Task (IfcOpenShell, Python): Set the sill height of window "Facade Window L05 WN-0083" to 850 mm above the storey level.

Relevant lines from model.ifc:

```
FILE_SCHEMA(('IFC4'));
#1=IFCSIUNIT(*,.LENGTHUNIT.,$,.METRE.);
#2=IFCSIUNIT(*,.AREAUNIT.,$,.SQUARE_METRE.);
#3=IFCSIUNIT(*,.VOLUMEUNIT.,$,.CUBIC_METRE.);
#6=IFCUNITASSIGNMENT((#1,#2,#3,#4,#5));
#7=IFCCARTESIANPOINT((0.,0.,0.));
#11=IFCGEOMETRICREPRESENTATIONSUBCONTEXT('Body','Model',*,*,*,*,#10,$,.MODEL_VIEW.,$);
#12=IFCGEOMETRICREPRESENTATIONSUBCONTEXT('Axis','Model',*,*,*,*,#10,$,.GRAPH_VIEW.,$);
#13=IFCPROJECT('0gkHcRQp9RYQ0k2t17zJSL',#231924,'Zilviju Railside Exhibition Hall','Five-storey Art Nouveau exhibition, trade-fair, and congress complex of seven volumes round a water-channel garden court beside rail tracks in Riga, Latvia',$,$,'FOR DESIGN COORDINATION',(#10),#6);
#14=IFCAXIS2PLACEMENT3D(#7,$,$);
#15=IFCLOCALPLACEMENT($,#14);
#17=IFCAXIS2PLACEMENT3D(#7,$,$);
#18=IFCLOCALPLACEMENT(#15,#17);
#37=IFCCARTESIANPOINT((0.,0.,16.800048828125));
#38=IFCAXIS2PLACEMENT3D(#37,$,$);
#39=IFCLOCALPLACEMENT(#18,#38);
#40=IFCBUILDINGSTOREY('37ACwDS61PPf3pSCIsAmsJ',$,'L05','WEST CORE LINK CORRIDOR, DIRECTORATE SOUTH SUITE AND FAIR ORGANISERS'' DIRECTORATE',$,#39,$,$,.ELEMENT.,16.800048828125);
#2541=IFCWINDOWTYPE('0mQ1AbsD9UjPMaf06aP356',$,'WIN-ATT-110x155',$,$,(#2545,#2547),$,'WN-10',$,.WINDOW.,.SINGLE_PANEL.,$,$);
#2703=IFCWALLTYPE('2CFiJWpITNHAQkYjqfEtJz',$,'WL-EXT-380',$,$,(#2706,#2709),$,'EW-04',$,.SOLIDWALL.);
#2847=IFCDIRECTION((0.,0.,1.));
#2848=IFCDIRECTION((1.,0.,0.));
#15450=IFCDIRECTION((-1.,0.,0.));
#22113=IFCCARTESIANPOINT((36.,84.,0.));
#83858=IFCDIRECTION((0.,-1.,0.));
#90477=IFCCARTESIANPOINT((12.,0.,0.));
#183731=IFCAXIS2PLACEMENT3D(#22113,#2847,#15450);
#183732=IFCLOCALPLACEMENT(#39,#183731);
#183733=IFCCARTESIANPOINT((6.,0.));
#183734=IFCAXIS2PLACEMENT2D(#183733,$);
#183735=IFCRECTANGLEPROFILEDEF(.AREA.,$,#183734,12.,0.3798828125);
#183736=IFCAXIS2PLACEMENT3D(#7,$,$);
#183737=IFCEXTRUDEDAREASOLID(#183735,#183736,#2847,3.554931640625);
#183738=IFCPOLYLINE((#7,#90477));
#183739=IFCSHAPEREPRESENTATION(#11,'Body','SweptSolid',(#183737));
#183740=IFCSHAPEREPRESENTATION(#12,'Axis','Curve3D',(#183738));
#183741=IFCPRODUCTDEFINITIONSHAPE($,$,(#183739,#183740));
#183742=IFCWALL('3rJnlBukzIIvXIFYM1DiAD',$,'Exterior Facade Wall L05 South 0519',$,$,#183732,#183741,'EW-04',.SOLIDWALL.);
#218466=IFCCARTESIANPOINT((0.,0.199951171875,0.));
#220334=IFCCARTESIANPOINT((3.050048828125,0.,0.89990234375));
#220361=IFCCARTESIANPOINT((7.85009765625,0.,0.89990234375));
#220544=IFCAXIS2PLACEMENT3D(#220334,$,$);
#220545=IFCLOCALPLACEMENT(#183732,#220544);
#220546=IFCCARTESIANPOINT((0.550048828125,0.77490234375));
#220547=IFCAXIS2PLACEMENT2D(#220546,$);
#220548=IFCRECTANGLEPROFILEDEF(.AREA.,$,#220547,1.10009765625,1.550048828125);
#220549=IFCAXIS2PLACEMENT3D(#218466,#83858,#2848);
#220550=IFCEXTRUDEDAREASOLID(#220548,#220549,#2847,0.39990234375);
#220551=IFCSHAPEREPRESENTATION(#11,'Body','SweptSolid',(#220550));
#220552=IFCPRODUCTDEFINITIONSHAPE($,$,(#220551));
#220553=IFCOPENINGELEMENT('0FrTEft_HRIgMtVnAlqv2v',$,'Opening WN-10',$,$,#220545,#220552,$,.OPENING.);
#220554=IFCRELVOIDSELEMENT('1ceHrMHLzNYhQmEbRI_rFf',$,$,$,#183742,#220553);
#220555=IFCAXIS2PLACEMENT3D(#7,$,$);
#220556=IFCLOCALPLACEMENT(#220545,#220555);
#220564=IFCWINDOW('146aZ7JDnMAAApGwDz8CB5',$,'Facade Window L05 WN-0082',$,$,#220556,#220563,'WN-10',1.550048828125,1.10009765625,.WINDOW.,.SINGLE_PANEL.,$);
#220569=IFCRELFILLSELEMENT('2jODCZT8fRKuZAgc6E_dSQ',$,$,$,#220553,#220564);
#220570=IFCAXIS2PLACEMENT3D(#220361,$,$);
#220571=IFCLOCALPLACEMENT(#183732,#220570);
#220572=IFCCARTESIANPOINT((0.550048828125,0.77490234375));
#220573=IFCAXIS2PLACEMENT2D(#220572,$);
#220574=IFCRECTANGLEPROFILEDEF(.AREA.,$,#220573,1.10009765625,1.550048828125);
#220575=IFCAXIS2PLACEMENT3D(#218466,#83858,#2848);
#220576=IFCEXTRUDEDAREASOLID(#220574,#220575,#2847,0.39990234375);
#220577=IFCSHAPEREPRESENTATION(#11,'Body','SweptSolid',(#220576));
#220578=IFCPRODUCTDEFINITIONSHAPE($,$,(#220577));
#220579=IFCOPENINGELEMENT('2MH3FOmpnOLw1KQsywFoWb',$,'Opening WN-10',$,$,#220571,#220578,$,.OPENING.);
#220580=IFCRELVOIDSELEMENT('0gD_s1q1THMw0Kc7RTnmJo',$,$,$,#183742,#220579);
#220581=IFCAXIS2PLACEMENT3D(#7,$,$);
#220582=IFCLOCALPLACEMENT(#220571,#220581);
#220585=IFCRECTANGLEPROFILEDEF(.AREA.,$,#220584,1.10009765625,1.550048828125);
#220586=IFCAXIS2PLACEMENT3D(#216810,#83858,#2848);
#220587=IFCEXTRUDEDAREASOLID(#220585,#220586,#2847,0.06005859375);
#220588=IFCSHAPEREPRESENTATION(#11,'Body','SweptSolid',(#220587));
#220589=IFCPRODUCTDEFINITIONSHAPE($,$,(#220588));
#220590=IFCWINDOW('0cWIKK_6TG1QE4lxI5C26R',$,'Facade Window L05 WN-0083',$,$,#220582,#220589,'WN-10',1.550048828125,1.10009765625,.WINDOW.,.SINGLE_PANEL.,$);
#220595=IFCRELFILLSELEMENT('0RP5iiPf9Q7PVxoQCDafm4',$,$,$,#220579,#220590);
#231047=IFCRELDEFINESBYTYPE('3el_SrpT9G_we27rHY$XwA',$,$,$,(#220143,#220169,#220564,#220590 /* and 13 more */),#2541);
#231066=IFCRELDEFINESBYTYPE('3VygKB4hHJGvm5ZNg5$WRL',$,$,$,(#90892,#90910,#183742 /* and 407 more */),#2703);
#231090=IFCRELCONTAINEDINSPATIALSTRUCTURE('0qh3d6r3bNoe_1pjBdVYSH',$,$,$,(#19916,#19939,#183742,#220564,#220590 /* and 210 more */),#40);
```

```python
import numpy as np
import ifcopenshell
import ifcopenshell.api.geometry
import ifcopenshell.geom
import ifcopenshell.util.element
import ifcopenshell.util.placement
import ifcopenshell.util.shape
import ifcopenshell.util.unit

model = ifcopenshell.open("model.ifc")
unit_scale = ifcopenshell.util.unit.calculate_unit_scale(model)

window = model.by_guid("0cWIKK_6TG1QE4lxI5C26R")
opening = window.FillsVoids[0].RelatingOpeningElement
storey = ifcopenshell.util.element.get_container(window, ifc_class="IfcBuildingStorey")
level = ifcopenshell.util.placement.get_local_placement(storey.ObjectPlacement)[2, 3]

# The opening's origin need not be at the sill, so measure its lowest point.
shape = ifcopenshell.geom.create_shape(ifcopenshell.geom.settings(), opening)
bottom = ifcopenshell.util.shape.get_shape_bottom_elevation(shape, shape.geometry) / unit_scale
dz = level + 0.85 / unit_scale - bottom

shift = np.array([0.0, 0.0, dz])
# The window is placed relative to its opening, so it follows when the opening moves.
matrix = ifcopenshell.util.placement.get_local_placement(opening.ObjectPlacement)
matrix[:3, 3] += shift
ifcopenshell.api.geometry.edit_object_placement(
    model, product=opening, matrix=matrix, is_si=False, should_transform_children=True
)

print(f"moved by {dz * unit_scale:+.3f} m")

model.write("model_v2.ifc")
```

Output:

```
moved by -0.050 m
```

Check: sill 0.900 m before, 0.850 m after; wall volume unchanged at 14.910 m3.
